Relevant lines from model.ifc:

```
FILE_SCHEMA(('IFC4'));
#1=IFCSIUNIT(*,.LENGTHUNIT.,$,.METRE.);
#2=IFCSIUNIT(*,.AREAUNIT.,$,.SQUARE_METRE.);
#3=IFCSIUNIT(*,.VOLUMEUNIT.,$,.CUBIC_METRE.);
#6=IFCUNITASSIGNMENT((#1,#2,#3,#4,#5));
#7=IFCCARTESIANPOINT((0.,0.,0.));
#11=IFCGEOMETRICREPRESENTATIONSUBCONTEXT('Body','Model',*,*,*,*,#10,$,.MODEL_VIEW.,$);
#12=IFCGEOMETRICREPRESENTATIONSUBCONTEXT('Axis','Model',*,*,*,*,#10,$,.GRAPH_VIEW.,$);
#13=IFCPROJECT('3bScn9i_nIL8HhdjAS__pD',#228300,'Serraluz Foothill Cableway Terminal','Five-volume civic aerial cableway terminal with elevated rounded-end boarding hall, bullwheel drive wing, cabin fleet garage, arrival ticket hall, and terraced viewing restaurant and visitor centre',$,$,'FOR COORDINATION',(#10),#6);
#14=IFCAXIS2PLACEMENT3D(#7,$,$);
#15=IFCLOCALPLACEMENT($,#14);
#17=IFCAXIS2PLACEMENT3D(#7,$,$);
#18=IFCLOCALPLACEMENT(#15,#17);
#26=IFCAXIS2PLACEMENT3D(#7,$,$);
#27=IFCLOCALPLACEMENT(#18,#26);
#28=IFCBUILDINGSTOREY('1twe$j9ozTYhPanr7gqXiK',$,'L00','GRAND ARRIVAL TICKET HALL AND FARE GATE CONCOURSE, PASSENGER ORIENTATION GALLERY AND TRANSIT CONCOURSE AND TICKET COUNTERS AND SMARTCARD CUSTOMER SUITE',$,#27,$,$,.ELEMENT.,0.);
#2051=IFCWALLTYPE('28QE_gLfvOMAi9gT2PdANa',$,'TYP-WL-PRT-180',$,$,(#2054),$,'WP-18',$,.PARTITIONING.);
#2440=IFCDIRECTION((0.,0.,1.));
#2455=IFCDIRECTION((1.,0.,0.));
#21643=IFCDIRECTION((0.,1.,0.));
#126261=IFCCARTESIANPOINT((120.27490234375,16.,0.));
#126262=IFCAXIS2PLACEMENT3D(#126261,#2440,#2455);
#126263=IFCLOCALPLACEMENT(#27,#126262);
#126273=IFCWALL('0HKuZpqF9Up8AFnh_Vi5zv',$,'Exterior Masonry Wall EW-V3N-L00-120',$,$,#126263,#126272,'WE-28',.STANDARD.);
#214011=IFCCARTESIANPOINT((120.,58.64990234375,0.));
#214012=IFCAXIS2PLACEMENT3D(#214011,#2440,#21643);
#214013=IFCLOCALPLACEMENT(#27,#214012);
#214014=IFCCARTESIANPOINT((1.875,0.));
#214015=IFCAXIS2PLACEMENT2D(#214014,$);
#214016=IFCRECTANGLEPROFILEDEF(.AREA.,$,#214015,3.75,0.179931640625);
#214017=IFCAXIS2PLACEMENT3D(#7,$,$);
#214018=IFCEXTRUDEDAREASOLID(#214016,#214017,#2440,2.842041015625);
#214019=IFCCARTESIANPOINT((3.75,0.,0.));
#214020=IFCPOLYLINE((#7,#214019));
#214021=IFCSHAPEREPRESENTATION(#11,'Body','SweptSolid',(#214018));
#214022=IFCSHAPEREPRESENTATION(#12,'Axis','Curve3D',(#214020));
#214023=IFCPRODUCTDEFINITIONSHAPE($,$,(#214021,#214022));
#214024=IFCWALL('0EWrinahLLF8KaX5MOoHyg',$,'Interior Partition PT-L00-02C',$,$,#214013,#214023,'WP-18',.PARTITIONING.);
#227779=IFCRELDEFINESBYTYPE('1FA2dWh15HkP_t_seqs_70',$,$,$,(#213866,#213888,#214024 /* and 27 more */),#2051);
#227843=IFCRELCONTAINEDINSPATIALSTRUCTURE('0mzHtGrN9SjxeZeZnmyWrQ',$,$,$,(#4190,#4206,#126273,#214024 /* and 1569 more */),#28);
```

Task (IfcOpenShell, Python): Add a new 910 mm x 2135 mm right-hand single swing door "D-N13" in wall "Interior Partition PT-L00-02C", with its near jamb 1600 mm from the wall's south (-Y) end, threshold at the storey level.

```python
import numpy as np
import ifcopenshell
import ifcopenshell.api.feature
import ifcopenshell.api.geometry
import ifcopenshell.api.root
import ifcopenshell.api.spatial
import ifcopenshell.geom
import ifcopenshell.util.element
import ifcopenshell.util.placement
import ifcopenshell.util.representation
import ifcopenshell.util.shape
import ifcopenshell.util.unit

model = ifcopenshell.open("model.ifc")
unit_scale = ifcopenshell.util.unit.calculate_unit_scale(model)
settings = ifcopenshell.geom.settings()


def volume(element):
    """Net volume in cubic metres, openings subtracted."""
    shape = ifcopenshell.geom.create_shape(settings, element)
    return ifcopenshell.util.shape.get_volume(shape.geometry)


wall = model.by_guid("0EWrinahLLF8KaX5MOoHyg")
storey = ifcopenshell.util.element.get_container(wall, ifc_class="IfcBuildingStorey")
context = ifcopenshell.util.representation.get_context(model, "Model", "Body", "MODEL_VIEW")
before = volume(wall)

width, height, from_end, sill = 0.91, 2.135, 1.6, 0.0  # metres

# The wall runs along its own X axis, and the end named is its -X end.
wall_shape = ifcopenshell.geom.create_shape(settings, wall)
x, y, z = ifcopenshell.util.shape.get_vertices(wall_shape.geometry).T
start = x.min() + from_end
face, thickness = float(y.min()), float(y.max() - y.min())
wall_matrix = ifcopenshell.util.placement.get_local_placement(wall.ObjectPlacement)
level = ifcopenshell.util.placement.get_local_placement(storey.ObjectPlacement)[2, 3]


def in_wall(x, y):
    """Placement at x, y metres in the wall's axes, at sill height."""
    matrix = wall_matrix.copy()
    matrix[:, 3] = wall_matrix @ np.array([x / unit_scale, y / unit_scale, 0.0, 1.0])
    matrix[2, 3] = level + sill / unit_scale
    return matrix


# Opening: a box that overshoots both wall faces by 50 mm.
opening = ifcopenshell.api.root.create_entity(model, ifc_class="IfcOpeningElement", predefined_type="OPENING")
box = ifcopenshell.api.geometry.add_wall_representation(
    model, context=context, length=width, height=height, thickness=thickness + 0.1
)
ifcopenshell.api.geometry.assign_representation(model, product=opening, representation=box)
ifcopenshell.api.geometry.edit_object_placement(model, product=opening, matrix=in_wall(start, face - 0.05), is_si=False)
ifcopenshell.api.feature.add_feature(model, feature=opening, element=wall)

door = ifcopenshell.api.root.create_entity(model, ifc_class="IfcDoor", name="D-N13", predefined_type="DOOR")
door.OverallWidth, door.OverallHeight = width / unit_scale, height / unit_scale
door.OperationType = "SINGLE_SWING_RIGHT"
body = ifcopenshell.api.geometry.add_door_representation(
    model,
    context=context,
    overall_width=door.OverallWidth,
    overall_height=door.OverallHeight,
    operation_type="SINGLE_SWING_RIGHT",
    lining_properties={"LiningDepth": thickness / unit_scale, "ThresholdDepth": thickness / unit_scale},
)
ifcopenshell.api.geometry.assign_representation(model, product=door, representation=body)
ifcopenshell.api.spatial.assign_container(model, products=[door], relating_structure=storey)
ifcopenshell.api.feature.add_filling(model, opening=opening, element=door)

# The lining spans the wall, so the door starts at the wall face.
ifcopenshell.api.geometry.edit_object_placement(model, product=door, matrix=in_wall(start, face), is_si=False)

after = volume(wall)

print(f"wall volume {before:.3f} -> {after:.3f} m3")

model.write("model-out.ifc")
```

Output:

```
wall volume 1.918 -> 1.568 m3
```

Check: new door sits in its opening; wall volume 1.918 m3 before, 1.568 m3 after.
